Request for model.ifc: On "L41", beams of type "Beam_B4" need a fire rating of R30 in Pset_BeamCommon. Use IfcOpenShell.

First a look at what the model holds.

```python
import ifcopenshell
import ifcopenshell.util.element

model = ifcopenshell.open("model.ifc")
print(model.schema)
storey = next(s for s in model.by_type("IfcBuildingStorey") if s.Name == "L41")
beams = [e for e in ifcopenshell.util.element.get_decomposition(storey) if e.is_a("IfcBeam")]
seen = {}
for e in beams:
    element_type = ifcopenshell.util.element.get_type(e)
    key = (element_type.Name if element_type != e and element_type else None, ifcopenshell.util.element.get_pset(e, "Pset_BeamCommon", "FireRating"))
    seen[key] = seen.get(key, 0) + 1
for (name, value), count in sorted(seen.items(), key=str):
    print(count, "x", name, "|", value)
```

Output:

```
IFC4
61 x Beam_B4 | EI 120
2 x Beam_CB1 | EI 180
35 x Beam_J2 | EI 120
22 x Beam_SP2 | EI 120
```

```python
import ifcopenshell
import ifcopenshell.api.pset
import ifcopenshell.util.element

model = ifcopenshell.open("model.ifc")

storey = next(s for s in model.by_type("IfcBuildingStorey") if s.Name == "L41")
beams = [e for e in ifcopenshell.util.element.get_decomposition(storey) if e.is_a("IfcBeam")]

count = 0
for e in beams:
    element_type = ifcopenshell.util.element.get_type(e)
    if element_type in (None, e) or element_type.Name != "Beam_B4":
        continue
    found = ifcopenshell.util.element.get_pset(e, "Pset_BeamCommon", should_inherit=False)
    if found:
        pset = model.by_id(found["id"])
        if len(ifcopenshell.util.element.get_elements_by_pset(pset)) > 1:
            pset = ifcopenshell.api.pset.unshare_pset(model, products=[e], pset=pset)[0]
    else:
        pset = ifcopenshell.api.pset.add_pset(model, product=e, name="Pset_BeamCommon")
    ifcopenshell.api.pset.edit_pset(model, pset=pset, properties={"FireRating": "R30"})
    count += 1

print(count, "beams updated")

model.write("model-out.ifc")
```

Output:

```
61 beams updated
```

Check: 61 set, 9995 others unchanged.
